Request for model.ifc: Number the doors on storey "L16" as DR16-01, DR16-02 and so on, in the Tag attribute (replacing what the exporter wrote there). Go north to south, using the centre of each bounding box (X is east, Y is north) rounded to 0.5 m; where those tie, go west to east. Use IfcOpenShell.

First a look at what the model holds.

```python
import ifcopenshell
import ifcopenshell.util.element
import ifcopenshell.util.placement

model = ifcopenshell.open("model.ifc")
print(model.schema)
storey = next(s for s in model.by_type("IfcBuildingStorey") if s.Name == "L16")
doors = [e for e in ifcopenshell.util.element.get_decomposition(storey) if e.is_a("IfcDoor")]
for e in sorted(doors, key=lambda e: e.id()):
    origin = ifcopenshell.util.placement.get_local_placement(e.ObjectPlacement)[:3, 3]
    print(e.id(), e.Tag, e.Name, origin.round(2) + 0.0, sep=" | ")
```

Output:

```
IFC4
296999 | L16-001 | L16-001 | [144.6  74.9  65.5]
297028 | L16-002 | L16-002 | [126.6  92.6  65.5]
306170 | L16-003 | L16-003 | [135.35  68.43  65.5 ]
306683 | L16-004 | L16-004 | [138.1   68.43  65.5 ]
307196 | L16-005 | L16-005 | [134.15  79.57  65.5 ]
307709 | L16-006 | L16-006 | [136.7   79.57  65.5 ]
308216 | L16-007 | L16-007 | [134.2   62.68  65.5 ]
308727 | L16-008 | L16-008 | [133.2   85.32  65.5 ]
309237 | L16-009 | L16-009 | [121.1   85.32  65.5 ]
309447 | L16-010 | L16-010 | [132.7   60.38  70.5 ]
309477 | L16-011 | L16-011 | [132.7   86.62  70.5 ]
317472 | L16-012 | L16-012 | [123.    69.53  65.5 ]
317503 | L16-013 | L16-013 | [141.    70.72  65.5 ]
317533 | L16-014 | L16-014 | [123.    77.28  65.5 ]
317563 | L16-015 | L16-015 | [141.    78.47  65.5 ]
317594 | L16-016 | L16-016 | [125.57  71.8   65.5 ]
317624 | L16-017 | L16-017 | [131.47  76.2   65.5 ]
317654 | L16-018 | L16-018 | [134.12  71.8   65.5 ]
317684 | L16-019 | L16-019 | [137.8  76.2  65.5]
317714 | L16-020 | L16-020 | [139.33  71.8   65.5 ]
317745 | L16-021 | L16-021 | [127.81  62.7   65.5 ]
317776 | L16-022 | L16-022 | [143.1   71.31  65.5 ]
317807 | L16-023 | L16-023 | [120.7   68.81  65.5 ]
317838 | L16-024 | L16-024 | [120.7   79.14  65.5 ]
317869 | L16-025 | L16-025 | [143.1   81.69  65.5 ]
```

```python
import ifcopenshell
import ifcopenshell.geom
import ifcopenshell.util.element
import ifcopenshell.util.shape

model = ifcopenshell.open("model.ifc")
settings = ifcopenshell.geom.settings()
settings.set("use-world-coords", True)


def centre(element):
    shape = ifcopenshell.geom.create_shape(settings, element)
    return ifcopenshell.util.shape.get_bbox_centroid(shape.geometry)


storey = next(s for s in model.by_type("IfcBuildingStorey") if s.Name == "L16")
doors = [e for e in ifcopenshell.util.element.get_decomposition(storey) if e.is_a("IfcDoor")]

# Insertion points can sit at a corner or the storey origin, so sort by the geometry (in metres).
centres = {e: centre(e) for e in doors}
doors.sort(key=lambda e: (-round(centres[e][1] / 0.5), centres[e][0]))

for i, e in enumerate(doors, start=1):
    number = f"DR16-{i:02d}"
    e.Tag = number
    print(e.id(), number)

model.write("model_v2.ifc")
```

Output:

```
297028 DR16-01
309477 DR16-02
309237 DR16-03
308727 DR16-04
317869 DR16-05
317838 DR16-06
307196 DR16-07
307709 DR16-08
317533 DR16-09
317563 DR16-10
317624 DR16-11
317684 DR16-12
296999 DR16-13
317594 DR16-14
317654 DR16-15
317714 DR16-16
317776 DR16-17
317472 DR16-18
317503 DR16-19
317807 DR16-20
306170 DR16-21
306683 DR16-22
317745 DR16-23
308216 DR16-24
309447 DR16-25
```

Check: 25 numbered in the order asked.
